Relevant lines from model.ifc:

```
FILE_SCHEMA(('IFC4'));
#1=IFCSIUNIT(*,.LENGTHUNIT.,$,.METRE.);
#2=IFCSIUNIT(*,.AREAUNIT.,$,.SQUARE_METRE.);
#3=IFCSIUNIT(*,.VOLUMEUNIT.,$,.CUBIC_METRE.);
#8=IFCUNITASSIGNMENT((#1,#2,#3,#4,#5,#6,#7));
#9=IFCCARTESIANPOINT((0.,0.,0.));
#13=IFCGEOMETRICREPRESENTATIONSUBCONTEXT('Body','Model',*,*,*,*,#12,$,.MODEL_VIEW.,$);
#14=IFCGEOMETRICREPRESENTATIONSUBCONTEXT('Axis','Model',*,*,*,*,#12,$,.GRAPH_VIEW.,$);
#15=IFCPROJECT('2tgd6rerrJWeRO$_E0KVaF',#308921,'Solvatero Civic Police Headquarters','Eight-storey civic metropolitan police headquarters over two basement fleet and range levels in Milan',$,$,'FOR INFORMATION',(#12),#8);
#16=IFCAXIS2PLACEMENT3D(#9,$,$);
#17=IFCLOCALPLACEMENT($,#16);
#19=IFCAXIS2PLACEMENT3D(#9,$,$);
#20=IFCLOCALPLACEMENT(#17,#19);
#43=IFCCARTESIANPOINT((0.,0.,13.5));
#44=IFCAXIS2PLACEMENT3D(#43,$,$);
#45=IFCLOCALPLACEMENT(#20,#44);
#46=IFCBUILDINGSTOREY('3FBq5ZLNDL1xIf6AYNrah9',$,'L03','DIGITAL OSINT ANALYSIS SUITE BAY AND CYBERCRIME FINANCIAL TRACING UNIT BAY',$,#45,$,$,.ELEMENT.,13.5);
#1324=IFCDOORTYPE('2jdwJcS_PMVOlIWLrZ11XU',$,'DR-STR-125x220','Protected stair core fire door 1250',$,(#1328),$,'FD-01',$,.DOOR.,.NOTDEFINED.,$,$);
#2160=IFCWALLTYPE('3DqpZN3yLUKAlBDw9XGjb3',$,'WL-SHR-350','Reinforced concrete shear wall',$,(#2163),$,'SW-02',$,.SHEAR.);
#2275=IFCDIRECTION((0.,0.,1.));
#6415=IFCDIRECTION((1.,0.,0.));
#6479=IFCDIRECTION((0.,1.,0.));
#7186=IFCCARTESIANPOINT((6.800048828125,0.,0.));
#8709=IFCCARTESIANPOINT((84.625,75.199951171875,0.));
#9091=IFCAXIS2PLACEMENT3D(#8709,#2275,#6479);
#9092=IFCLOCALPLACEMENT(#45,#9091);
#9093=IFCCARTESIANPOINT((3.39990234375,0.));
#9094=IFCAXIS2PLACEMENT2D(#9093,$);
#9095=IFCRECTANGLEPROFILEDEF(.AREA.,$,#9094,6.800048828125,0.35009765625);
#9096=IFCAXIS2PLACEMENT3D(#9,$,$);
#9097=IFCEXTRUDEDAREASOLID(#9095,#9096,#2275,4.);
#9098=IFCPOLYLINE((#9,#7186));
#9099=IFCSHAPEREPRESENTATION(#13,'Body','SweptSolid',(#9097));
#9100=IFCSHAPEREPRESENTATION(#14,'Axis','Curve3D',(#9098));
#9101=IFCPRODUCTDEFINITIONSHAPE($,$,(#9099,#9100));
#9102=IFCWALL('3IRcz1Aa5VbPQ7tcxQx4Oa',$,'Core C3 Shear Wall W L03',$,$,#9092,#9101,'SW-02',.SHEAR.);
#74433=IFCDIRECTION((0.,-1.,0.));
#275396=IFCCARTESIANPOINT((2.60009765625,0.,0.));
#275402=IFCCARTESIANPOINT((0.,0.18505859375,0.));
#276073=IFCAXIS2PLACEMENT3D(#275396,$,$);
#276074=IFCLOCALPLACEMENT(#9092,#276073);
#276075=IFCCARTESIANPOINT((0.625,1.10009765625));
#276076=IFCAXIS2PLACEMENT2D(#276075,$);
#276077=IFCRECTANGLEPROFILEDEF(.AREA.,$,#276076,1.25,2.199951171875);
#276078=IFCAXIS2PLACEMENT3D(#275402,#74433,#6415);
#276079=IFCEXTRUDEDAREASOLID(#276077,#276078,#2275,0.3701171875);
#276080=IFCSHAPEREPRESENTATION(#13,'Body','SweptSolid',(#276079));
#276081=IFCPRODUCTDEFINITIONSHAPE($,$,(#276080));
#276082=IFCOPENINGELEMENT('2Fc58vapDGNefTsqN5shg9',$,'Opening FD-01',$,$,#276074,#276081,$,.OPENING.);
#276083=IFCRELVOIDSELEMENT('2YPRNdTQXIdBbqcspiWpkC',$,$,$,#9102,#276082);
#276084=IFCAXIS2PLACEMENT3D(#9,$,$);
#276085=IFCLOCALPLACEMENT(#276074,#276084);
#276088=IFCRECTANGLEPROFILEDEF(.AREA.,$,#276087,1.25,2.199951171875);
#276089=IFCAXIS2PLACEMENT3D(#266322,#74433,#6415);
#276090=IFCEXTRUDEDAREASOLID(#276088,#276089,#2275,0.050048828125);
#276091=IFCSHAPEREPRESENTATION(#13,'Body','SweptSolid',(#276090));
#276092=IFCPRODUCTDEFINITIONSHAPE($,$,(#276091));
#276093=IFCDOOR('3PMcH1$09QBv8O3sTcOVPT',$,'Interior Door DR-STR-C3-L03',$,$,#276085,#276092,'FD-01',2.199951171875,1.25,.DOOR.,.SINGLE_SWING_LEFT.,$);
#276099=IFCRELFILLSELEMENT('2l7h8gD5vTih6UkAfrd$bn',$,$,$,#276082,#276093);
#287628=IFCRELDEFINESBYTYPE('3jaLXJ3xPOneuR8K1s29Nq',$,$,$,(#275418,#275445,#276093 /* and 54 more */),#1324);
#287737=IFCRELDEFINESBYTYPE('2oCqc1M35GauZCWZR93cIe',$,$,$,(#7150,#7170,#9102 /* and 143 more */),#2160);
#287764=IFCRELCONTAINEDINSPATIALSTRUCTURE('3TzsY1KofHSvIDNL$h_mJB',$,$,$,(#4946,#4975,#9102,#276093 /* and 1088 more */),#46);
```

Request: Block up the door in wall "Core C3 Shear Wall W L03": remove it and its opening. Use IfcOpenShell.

```python
import ifcopenshell
import ifcopenshell.api.feature
import ifcopenshell.api.root
import ifcopenshell.geom
import ifcopenshell.util.shape

model = ifcopenshell.open("model.ifc")
settings = ifcopenshell.geom.settings()


def volume(element):
    """Net volume in cubic metres, openings subtracted."""
    shape = ifcopenshell.geom.create_shape(settings, element)
    return ifcopenshell.util.shape.get_volume(shape.geometry)


door = model.by_guid("3PMcH1$09QBv8O3sTcOVPT")
opening = door.FillsVoids[0].RelatingOpeningElement
wall = opening.VoidsElements[0].RelatingBuildingElement
before = volume(wall)

ifcopenshell.api.root.remove_product(model, product=door)
ifcopenshell.api.feature.remove_feature(model, feature=opening)

after = volume(wall)

print(f"wall volume {before:.3f} -> {after:.3f} m3")

model.write("model-out.ifc")
```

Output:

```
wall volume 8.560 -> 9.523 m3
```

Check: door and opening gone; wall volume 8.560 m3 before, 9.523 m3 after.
